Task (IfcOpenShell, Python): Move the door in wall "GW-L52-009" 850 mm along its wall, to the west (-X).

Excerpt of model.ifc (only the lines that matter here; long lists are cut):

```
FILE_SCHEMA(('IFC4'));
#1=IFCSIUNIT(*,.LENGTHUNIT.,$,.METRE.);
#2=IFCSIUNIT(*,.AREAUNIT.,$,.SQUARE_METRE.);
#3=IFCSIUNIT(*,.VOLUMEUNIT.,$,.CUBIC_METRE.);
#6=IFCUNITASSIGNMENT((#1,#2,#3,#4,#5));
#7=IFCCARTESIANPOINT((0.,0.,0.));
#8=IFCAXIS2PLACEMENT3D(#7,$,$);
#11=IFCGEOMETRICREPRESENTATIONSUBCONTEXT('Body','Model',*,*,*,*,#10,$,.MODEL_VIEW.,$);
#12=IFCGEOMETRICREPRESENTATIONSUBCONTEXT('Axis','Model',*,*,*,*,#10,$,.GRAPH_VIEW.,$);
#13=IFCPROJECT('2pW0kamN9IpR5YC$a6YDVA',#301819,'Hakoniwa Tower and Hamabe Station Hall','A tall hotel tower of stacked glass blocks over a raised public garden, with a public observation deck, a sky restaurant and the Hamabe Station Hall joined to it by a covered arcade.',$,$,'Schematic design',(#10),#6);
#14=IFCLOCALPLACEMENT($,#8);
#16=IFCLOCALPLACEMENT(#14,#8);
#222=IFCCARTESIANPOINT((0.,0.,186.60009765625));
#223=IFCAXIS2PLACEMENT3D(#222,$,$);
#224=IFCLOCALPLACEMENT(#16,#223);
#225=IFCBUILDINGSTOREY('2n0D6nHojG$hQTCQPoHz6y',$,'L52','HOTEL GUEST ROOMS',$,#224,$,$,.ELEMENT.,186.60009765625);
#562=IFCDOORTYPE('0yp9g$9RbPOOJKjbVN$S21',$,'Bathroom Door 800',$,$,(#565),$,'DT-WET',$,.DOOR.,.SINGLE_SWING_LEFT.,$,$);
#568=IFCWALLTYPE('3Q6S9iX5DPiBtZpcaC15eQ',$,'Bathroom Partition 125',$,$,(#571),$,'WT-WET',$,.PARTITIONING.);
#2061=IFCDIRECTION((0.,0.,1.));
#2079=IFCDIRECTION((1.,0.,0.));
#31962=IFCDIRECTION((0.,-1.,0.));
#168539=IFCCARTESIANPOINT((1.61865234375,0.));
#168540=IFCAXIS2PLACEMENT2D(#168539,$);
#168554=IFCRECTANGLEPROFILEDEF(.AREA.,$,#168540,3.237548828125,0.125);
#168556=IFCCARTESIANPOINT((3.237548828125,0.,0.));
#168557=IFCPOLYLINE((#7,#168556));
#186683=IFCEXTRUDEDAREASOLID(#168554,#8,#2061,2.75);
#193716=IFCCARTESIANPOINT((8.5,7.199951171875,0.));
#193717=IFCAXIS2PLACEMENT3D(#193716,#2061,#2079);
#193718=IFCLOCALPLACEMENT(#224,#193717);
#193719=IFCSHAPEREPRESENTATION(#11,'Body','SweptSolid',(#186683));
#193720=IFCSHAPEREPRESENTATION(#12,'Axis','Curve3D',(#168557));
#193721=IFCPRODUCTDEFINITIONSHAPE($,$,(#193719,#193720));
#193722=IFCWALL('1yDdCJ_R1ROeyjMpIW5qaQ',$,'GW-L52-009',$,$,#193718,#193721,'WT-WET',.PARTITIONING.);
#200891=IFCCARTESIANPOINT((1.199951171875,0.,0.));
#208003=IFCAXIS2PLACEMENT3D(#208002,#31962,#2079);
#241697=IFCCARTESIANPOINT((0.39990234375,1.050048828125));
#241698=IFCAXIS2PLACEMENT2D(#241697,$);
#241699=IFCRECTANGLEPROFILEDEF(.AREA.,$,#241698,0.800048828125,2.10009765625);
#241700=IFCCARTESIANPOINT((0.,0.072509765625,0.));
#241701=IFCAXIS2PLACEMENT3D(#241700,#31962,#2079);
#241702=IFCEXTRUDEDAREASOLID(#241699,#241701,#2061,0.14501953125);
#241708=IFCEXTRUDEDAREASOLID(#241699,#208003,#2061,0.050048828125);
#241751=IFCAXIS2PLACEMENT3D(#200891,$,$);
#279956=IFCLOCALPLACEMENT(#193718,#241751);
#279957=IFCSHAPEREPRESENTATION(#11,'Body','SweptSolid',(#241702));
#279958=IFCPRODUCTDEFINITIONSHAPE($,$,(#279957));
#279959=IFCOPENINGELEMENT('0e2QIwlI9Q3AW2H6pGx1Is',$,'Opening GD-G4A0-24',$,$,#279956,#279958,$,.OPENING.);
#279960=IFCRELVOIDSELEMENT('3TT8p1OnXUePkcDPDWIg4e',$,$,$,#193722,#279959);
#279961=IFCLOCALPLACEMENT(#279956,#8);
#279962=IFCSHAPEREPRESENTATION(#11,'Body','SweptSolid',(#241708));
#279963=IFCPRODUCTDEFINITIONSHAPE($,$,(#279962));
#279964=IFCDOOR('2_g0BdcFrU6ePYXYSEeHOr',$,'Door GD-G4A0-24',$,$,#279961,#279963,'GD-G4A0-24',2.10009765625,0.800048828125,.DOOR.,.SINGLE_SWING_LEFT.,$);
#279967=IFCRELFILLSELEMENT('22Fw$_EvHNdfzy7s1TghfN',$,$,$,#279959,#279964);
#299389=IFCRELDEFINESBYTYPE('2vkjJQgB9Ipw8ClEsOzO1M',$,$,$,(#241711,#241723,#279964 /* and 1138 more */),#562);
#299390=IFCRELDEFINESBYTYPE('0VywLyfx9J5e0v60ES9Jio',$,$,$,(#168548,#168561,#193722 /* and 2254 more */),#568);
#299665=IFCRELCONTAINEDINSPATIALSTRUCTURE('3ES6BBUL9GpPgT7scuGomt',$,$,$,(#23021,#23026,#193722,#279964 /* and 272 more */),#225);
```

```python
import ifcopenshell
import ifcopenshell.api.geometry
import ifcopenshell.util.placement
import ifcopenshell.util.unit

model = ifcopenshell.open("model.ifc")
unit_scale = ifcopenshell.util.unit.calculate_unit_scale(model)

door = model.by_guid("2_g0BdcFrU6ePYXYSEeHOr")
opening = door.FillsVoids[0].RelatingOpeningElement
wall = opening.VoidsElements[0].RelatingBuildingElement

wall_matrix = ifcopenshell.util.placement.get_local_placement(wall.ObjectPlacement)
shift = wall_matrix[:3, 0] * -0.85 / unit_scale
before = ifcopenshell.util.placement.get_local_placement(door.ObjectPlacement)[:3, 3].copy()

# The door is placed relative to its opening, so it follows when the opening moves.
matrix = ifcopenshell.util.placement.get_local_placement(opening.ObjectPlacement)
matrix[:3, 3] += shift
ifcopenshell.api.geometry.edit_object_placement(
    model, product=opening, matrix=matrix, is_si=False, should_transform_children=True
)

after = ifcopenshell.util.placement.get_local_placement(door.ObjectPlacement)[:3, 3]
print("door moved by", (after - before).round(3) + 0.0)

model.write("model-out.ifc")
```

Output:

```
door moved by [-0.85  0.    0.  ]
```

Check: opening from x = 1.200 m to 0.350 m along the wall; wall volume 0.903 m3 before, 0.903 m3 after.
